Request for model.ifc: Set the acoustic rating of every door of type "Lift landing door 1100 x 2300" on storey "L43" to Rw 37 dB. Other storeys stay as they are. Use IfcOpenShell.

First a look at what the model holds.

```python
import ifcopenshell
import ifcopenshell.util.element

model = ifcopenshell.open("model.ifc")
print(model.schema)
storey = next(s for s in model.by_type("IfcBuildingStorey") if s.Name == "L43")
doors = [e for e in ifcopenshell.util.element.get_decomposition(storey) if e.is_a("IfcDoor")]
seen = {}
for e in doors:
    element_type = ifcopenshell.util.element.get_type(e)
    key = (element_type.Name if element_type != e and element_type else None, ifcopenshell.util.element.get_pset(e, "Pset_DoorCommon", "AcousticRating"))
    seen[key] = seen.get(key, 0) + 1
for (name, value), count in sorted(seen.items(), key=str):
    print(count, "x", name, "|", value)
```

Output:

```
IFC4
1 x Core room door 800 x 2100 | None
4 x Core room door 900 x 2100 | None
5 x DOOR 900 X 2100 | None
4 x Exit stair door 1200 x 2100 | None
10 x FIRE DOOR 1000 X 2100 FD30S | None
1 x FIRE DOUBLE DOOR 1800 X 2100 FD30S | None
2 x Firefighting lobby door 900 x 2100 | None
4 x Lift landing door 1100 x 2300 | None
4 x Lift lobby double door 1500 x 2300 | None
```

```python
import ifcopenshell
import ifcopenshell.api.pset
import ifcopenshell.util.element

model = ifcopenshell.open("model.ifc")

storey = next(s for s in model.by_type("IfcBuildingStorey") if s.Name == "L43")
doors = [e for e in ifcopenshell.util.element.get_decomposition(storey) if e.is_a("IfcDoor")]

count = 0
for e in doors:
    element_type = ifcopenshell.util.element.get_type(e)
    if element_type in (None, e) or element_type.Name != "Lift landing door 1100 x 2300":
        continue
    found = ifcopenshell.util.element.get_pset(e, "Pset_DoorCommon", should_inherit=False)
    if found:
        pset = model.by_id(found["id"])
        if len(ifcopenshell.util.element.get_elements_by_pset(pset)) > 1:
            pset = ifcopenshell.api.pset.unshare_pset(model, products=[e], pset=pset)[0]
    else:
        pset = ifcopenshell.api.pset.add_pset(model, product=e, name="Pset_DoorCommon")
    ifcopenshell.api.pset.edit_pset(model, pset=pset, properties={"AcousticRating": "Rw 37 dB"})
    count += 1

print(count, "doors updated")

model.write("model_updated.ifc")
```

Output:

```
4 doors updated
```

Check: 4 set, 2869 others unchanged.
